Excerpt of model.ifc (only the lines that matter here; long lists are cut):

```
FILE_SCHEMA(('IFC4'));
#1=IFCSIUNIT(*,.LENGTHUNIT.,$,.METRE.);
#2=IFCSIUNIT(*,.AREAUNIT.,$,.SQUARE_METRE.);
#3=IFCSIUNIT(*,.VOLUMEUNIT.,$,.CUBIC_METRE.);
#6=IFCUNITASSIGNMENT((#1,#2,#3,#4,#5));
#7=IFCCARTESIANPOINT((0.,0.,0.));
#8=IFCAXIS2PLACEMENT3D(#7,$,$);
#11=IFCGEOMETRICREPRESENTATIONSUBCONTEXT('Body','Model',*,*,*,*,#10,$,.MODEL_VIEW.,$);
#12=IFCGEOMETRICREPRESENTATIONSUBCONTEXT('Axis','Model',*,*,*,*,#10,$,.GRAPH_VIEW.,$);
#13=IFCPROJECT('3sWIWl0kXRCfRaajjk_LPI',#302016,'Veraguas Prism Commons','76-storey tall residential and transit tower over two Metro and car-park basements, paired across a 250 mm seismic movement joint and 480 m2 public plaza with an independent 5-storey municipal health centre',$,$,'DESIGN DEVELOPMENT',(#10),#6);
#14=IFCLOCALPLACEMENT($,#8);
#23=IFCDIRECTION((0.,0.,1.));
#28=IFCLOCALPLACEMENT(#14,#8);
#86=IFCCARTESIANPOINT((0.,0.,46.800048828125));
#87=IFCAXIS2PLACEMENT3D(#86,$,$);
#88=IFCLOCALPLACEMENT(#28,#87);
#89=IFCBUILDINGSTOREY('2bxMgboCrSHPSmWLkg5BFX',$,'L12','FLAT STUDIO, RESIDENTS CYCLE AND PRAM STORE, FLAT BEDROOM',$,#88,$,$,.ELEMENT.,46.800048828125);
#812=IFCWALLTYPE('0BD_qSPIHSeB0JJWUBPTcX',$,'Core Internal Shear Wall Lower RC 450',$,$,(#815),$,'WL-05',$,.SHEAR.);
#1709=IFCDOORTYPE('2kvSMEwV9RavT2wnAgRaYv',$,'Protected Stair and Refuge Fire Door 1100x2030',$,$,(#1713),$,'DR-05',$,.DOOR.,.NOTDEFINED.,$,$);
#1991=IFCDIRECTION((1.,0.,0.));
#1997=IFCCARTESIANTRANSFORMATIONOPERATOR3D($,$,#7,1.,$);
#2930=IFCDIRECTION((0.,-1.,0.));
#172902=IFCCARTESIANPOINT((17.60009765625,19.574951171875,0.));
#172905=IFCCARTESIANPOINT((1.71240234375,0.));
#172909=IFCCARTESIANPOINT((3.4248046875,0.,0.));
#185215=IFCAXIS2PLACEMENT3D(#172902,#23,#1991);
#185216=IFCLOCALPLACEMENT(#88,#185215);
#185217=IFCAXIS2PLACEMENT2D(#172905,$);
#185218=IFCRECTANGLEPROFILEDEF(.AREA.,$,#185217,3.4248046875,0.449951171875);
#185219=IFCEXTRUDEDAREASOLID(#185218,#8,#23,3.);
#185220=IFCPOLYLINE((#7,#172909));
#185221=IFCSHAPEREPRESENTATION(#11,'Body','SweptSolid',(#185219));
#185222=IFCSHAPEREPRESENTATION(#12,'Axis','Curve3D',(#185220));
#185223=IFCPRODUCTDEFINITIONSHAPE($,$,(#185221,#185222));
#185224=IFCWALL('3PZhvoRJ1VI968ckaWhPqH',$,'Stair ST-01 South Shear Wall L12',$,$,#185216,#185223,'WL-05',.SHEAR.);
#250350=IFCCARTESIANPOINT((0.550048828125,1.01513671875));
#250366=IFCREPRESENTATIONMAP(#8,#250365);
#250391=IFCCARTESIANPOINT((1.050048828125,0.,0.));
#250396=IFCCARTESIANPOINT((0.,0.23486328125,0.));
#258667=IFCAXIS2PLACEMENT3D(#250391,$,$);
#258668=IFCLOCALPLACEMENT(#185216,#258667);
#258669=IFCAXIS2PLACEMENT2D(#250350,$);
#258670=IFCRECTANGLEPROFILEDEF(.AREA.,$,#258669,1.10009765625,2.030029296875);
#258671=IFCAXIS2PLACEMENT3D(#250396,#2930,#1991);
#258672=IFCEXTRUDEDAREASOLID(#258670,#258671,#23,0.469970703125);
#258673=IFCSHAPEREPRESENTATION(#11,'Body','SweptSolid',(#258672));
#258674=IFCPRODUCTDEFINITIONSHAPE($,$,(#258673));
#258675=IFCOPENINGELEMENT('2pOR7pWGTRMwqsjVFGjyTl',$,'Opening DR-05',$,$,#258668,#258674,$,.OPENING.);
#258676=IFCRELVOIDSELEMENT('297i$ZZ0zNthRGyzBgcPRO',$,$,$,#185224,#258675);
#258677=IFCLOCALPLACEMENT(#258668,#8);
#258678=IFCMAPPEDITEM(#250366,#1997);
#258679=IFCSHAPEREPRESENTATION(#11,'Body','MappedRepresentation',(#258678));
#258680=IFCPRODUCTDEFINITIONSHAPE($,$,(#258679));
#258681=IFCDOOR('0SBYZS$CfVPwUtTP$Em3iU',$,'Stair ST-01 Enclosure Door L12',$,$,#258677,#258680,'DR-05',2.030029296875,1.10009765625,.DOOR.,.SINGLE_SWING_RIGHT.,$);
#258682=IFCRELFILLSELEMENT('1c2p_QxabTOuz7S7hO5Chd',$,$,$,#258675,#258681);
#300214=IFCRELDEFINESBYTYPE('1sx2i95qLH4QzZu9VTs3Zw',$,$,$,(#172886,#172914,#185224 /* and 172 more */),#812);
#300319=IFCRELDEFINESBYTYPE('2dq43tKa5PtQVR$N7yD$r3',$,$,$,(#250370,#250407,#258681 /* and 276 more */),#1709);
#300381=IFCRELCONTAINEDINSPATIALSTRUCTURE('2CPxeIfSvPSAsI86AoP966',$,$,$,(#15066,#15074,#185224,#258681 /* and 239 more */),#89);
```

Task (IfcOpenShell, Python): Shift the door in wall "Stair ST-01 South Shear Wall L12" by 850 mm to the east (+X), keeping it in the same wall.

```python
import ifcopenshell
import ifcopenshell.api.geometry
import ifcopenshell.util.placement

model = ifcopenshell.open("model.ifc")

door = model.by_guid("0SBYZS$CfVPwUtTP$Em3iU")
opening = door.FillsVoids[0].RelatingOpeningElement
wall = opening.VoidsElements[0].RelatingBuildingElement

wall_matrix = ifcopenshell.util.placement.get_local_placement(wall.ObjectPlacement)
shift = wall_matrix[:3, 0] * 0.85
before = ifcopenshell.util.placement.get_local_placement(door.ObjectPlacement)[:3, 3].copy()

# The door is placed relative to its opening, so it follows when the opening moves.
matrix = ifcopenshell.util.placement.get_local_placement(opening.ObjectPlacement)
matrix[:3, 3] += shift
ifcopenshell.api.geometry.edit_object_placement(
    model, product=opening, matrix=matrix, is_si=False, should_transform_children=True
)

after = ifcopenshell.util.placement.get_local_placement(door.ObjectPlacement)[:3, 3]
print("door moved by", (after - before).round(3) + 0.0)

model.write("model_v2.ifc")
```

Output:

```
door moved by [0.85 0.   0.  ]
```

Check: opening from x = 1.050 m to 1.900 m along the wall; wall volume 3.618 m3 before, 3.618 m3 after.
